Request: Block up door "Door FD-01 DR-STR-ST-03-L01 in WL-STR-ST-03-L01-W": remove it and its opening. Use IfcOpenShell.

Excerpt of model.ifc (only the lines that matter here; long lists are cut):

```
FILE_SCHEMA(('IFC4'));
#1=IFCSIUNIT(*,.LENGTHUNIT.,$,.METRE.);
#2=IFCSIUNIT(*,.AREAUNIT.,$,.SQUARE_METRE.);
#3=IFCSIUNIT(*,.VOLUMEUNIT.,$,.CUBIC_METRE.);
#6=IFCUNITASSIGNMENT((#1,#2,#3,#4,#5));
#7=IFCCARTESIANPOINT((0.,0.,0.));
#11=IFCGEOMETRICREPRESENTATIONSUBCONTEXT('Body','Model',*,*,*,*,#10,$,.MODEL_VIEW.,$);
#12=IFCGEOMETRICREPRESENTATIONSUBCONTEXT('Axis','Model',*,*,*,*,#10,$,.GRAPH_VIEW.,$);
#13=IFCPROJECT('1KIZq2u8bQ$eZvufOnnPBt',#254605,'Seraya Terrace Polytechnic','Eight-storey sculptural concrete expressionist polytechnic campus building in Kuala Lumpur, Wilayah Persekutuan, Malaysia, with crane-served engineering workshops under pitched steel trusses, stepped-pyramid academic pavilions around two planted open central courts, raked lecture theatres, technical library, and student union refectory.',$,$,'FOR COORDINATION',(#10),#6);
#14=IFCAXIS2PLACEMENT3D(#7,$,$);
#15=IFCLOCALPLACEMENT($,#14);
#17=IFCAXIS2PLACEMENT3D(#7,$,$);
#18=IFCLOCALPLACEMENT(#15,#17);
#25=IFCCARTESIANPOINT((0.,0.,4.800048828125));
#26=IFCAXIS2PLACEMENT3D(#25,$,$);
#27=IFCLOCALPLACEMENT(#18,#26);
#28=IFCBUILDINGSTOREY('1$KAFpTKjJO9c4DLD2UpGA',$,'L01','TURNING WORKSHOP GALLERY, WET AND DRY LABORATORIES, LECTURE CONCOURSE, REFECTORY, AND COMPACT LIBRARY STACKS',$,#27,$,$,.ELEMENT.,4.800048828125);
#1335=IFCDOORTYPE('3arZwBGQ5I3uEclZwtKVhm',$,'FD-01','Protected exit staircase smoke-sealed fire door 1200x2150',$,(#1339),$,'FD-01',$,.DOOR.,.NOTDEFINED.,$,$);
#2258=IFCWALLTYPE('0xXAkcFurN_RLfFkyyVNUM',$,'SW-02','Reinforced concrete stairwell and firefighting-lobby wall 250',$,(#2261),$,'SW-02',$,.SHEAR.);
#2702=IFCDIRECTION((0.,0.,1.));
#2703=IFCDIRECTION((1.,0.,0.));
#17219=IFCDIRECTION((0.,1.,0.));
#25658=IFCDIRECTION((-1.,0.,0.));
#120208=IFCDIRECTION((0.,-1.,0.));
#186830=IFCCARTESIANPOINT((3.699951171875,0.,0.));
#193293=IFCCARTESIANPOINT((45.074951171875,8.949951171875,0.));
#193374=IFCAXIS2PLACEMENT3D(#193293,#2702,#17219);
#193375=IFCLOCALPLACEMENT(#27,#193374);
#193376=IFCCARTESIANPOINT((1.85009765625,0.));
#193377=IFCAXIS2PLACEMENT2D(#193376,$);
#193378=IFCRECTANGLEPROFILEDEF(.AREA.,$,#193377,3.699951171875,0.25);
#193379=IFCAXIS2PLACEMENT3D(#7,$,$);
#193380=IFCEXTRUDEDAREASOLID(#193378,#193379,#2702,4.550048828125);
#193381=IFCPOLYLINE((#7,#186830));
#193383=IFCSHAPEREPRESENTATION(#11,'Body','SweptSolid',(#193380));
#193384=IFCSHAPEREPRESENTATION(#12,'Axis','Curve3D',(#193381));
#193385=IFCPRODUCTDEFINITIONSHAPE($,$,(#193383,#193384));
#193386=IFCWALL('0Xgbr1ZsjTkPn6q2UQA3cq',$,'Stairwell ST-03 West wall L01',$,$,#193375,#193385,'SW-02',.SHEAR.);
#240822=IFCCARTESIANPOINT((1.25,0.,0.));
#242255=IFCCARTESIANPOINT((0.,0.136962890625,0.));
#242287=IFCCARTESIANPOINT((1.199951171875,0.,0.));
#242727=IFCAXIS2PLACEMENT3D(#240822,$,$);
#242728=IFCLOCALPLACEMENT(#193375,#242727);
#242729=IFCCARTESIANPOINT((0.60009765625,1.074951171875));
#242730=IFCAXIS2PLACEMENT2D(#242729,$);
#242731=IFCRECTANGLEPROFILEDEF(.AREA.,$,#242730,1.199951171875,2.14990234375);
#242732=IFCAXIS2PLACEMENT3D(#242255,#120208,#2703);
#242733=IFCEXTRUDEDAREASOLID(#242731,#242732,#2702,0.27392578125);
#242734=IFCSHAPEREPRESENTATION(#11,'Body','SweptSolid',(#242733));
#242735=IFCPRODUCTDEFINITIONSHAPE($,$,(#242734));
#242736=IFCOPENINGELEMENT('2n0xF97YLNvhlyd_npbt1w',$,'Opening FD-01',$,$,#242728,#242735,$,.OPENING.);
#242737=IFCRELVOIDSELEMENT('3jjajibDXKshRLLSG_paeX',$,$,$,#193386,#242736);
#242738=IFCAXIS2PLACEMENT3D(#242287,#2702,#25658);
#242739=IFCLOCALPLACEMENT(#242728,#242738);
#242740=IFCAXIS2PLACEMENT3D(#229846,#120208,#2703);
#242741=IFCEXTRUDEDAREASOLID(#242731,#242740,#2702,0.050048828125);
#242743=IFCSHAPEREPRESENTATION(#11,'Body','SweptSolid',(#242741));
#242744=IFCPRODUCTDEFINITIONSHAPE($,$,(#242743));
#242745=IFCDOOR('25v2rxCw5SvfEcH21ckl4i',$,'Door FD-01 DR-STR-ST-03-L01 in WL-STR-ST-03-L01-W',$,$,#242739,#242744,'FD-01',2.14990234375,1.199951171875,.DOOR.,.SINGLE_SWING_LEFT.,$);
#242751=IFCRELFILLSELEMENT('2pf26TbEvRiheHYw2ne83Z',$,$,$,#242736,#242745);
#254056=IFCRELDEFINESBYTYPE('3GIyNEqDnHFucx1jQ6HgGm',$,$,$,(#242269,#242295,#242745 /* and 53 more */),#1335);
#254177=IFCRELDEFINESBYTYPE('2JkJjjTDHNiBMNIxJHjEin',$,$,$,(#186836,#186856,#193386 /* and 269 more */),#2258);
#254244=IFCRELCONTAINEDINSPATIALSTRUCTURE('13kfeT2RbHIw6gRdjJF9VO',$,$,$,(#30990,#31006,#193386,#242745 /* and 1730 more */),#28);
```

```python
import ifcopenshell
import ifcopenshell.api.feature
import ifcopenshell.api.root
import ifcopenshell.geom
import ifcopenshell.util.shape

model = ifcopenshell.open("model.ifc")
settings = ifcopenshell.geom.settings()


def volume(element):
    """Net volume in cubic metres, openings subtracted."""
    shape = ifcopenshell.geom.create_shape(settings, element)
    return ifcopenshell.util.shape.get_volume(shape.geometry)


door = model.by_guid("25v2rxCw5SvfEcH21ckl4i")
opening = door.FillsVoids[0].RelatingOpeningElement
wall = opening.VoidsElements[0].RelatingBuildingElement
before = volume(wall)

ifcopenshell.api.root.remove_product(model, product=door)
ifcopenshell.api.feature.remove_feature(model, feature=opening)

after = volume(wall)

print(f"wall volume {before:.3f} -> {after:.3f} m3")

model.write("model_v2.ifc")
```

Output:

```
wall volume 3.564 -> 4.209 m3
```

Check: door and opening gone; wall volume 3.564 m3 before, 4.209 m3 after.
